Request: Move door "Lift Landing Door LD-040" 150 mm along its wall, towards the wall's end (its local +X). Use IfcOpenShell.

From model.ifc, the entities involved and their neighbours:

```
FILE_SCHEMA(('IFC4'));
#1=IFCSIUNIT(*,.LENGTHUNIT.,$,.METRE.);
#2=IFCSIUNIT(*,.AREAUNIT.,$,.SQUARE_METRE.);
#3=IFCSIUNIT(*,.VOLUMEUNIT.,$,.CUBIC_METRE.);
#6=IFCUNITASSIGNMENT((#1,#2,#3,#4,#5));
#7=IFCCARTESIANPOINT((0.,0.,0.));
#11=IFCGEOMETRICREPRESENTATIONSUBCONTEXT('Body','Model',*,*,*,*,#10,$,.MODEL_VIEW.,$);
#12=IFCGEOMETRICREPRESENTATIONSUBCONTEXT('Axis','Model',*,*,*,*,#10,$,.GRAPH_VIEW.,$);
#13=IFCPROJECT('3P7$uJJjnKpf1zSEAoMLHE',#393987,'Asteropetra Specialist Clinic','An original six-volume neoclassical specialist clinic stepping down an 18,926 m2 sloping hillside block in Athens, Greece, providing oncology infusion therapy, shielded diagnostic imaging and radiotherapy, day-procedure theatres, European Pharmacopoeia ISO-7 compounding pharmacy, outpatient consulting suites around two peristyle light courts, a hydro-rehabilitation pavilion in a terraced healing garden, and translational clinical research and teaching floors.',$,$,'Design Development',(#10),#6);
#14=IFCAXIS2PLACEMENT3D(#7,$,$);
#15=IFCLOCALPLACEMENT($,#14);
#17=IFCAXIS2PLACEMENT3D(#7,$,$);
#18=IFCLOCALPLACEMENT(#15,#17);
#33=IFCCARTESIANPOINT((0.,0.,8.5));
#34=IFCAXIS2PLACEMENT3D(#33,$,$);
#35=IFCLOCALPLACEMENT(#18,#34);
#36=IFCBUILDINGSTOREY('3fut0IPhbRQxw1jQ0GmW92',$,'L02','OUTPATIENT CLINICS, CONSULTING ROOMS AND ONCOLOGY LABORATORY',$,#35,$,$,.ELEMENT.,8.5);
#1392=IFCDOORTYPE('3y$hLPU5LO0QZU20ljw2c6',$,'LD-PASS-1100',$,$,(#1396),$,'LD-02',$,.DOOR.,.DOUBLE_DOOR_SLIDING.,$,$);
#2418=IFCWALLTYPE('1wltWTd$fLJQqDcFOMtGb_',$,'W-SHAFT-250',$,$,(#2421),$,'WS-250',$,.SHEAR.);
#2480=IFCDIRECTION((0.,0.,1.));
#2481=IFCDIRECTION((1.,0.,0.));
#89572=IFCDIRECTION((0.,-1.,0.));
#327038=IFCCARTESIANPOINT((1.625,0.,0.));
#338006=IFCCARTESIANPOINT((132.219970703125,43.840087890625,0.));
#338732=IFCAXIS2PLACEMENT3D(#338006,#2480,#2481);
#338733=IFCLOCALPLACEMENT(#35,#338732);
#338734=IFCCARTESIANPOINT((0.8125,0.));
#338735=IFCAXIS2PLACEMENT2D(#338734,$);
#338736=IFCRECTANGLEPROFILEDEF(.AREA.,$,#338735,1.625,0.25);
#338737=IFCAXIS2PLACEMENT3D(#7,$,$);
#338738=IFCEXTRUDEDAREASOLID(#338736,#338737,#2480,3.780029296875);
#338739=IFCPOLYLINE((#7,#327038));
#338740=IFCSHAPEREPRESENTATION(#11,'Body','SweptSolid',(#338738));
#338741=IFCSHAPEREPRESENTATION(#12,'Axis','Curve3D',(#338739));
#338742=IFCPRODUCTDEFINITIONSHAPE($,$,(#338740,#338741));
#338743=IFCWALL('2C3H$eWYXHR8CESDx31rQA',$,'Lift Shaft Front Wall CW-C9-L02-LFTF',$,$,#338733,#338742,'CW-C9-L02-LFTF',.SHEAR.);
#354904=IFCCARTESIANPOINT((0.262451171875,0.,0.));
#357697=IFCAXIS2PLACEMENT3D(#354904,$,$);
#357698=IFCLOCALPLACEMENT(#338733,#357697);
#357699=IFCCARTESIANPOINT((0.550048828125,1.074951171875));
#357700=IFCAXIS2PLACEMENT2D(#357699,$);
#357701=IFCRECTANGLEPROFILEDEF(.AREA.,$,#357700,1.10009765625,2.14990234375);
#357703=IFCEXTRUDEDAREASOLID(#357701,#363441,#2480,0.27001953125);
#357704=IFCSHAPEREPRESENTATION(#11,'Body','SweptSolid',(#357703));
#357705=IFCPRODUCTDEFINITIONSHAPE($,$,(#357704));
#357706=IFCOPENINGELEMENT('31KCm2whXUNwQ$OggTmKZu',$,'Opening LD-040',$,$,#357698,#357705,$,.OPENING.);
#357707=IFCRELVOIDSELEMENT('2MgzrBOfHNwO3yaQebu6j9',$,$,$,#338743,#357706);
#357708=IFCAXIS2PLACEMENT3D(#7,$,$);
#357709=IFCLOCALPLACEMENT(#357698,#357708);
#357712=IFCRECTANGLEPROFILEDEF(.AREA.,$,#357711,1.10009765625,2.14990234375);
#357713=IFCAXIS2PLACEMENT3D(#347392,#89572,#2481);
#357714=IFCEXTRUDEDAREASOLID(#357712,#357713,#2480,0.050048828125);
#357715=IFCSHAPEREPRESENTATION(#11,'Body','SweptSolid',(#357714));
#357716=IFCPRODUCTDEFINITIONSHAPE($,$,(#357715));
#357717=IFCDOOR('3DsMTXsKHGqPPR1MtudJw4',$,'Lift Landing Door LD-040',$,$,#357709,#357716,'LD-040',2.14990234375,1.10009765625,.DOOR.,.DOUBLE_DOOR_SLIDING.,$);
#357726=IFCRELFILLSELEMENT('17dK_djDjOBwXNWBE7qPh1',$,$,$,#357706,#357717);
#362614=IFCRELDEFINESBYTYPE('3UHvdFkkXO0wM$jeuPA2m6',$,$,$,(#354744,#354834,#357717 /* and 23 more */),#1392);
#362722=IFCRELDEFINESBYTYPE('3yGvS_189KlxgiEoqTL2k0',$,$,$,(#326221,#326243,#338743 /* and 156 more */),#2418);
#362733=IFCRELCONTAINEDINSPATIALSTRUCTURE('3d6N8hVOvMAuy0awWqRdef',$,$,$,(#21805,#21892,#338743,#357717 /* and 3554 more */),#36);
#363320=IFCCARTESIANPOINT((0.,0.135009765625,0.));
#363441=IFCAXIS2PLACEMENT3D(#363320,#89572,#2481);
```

```python
import ifcopenshell
import ifcopenshell.api.geometry
import ifcopenshell.util.placement
import ifcopenshell.util.unit

model = ifcopenshell.open("model.ifc")
unit_scale = ifcopenshell.util.unit.calculate_unit_scale(model)

door = model.by_id(357717)
opening = door.FillsVoids[0].RelatingOpeningElement
wall = opening.VoidsElements[0].RelatingBuildingElement

wall_matrix = ifcopenshell.util.placement.get_local_placement(wall.ObjectPlacement)
shift = wall_matrix[:3, 0] * 0.15 / unit_scale
before = ifcopenshell.util.placement.get_local_placement(door.ObjectPlacement)[:3, 3].copy()

# The door is placed relative to its opening, so it follows when the opening moves.
matrix = ifcopenshell.util.placement.get_local_placement(opening.ObjectPlacement)
matrix[:3, 3] += shift
ifcopenshell.api.geometry.edit_object_placement(
    model, product=opening, matrix=matrix, is_si=False, should_transform_children=True
)

after = ifcopenshell.util.placement.get_local_placement(door.ObjectPlacement)[:3, 3]
print("door moved by", (after - before).round(3) + 0.0)

model.write("model_updated.ifc")
```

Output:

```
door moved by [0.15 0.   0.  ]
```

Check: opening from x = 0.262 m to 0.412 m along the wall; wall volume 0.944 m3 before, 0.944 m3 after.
